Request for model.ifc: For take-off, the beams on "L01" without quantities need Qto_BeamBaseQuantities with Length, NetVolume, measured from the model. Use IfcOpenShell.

First a look at what the model holds.

```python
import ifcopenshell
import ifcopenshell.util.element
import ifcopenshell.util.unit

model = ifcopenshell.open("model.ifc")
print(model.schema)
for unit_type in ("LENGTHUNIT", "AREAUNIT", "VOLUMEUNIT"):
    print(unit_type, ifcopenshell.util.unit.calculate_unit_scale(model, unit_type))
storey = next(s for s in model.by_type("IfcBuildingStorey") if s.Name == "L01")
beams = [e for e in ifcopenshell.util.element.get_decomposition(storey) if e.is_a("IfcBeam")]
for e in sorted(beams, key=lambda e: e.id()):
    print(e.id(), e.is_a(), e.Name, list(ifcopenshell.util.element.get_psets(e, qtos_only=True)), sep=" | ")
```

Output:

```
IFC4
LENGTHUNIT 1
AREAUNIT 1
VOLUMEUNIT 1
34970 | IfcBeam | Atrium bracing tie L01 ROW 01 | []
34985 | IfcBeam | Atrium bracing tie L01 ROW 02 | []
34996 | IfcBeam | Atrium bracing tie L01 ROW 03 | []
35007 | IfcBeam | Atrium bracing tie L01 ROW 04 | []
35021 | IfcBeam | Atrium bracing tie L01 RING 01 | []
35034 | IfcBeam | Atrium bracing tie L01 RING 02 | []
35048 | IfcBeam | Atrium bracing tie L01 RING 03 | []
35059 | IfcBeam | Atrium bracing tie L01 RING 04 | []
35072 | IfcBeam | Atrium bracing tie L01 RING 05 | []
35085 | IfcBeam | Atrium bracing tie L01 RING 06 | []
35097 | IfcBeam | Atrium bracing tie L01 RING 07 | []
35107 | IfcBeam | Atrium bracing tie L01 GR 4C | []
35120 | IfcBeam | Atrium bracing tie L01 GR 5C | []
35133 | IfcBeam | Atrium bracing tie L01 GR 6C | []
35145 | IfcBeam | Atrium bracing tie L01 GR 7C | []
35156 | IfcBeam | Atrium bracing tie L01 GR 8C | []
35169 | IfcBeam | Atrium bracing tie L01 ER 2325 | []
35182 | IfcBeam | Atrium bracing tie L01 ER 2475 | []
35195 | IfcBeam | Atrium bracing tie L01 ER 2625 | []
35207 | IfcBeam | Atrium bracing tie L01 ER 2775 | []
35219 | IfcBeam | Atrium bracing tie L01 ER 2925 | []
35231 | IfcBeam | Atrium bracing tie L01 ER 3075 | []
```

```python
import ifcopenshell
import ifcopenshell.api.pset
import ifcopenshell.geom
import ifcopenshell.util.element
import ifcopenshell.util.shape
import ifcopenshell.util.unit

model = ifcopenshell.open("model.ifc")
unit_scale = ifcopenshell.util.unit.calculate_unit_scale(model)
volume_scale = ifcopenshell.util.unit.calculate_unit_scale(model, "VOLUMEUNIT")
settings = ifcopenshell.geom.settings()

storey = next(s for s in model.by_type("IfcBuildingStorey") if s.Name == "L01")
beams = [e for e in ifcopenshell.util.element.get_decomposition(storey) if e.is_a("IfcBeam")]

for e in sorted(beams, key=lambda e: e.id()):
    if ifcopenshell.util.element.get_psets(e, qtos_only=True, should_inherit=False):
        continue
    # Geometry comes back in metres, in the element's own axes.
    shape = ifcopenshell.geom.create_shape(settings, e)
    values = {
        "Length": ifcopenshell.util.shape.get_max_xyz(shape.geometry) / unit_scale,
        "NetVolume": ifcopenshell.util.shape.get_volume(shape.geometry) / volume_scale,
    }
    qto = ifcopenshell.api.pset.add_qto(model, product=e, name="Qto_BeamBaseQuantities")
    ifcopenshell.api.pset.edit_qto(model, qto=qto, properties=values)
    print(e.id(), {k: round(v, 3) for k, v in values.items()})

model.write("model-out.ifc")
```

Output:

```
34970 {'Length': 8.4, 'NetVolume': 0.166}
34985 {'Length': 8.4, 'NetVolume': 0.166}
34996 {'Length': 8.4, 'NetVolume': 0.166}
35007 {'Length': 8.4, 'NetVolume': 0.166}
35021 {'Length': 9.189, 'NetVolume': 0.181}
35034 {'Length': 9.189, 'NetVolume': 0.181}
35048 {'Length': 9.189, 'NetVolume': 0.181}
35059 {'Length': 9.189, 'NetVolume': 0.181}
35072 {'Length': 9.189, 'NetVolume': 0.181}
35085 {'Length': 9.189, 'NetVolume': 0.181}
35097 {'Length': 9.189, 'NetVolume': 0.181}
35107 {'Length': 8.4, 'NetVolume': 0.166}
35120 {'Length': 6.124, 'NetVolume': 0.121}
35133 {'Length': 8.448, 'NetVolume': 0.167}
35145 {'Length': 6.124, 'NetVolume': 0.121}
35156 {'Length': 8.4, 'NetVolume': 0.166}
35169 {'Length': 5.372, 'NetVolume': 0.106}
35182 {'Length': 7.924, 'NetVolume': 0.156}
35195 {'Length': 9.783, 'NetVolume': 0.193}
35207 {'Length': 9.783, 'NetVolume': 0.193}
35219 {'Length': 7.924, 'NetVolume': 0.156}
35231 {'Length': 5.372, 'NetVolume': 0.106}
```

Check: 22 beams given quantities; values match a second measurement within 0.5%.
